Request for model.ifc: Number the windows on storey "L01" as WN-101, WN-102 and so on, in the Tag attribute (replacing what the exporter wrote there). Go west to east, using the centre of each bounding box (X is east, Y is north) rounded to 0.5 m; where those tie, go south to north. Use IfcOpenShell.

First a look at what the model holds.

```python
import ifcopenshell
import ifcopenshell.util.element
import ifcopenshell.util.placement

model = ifcopenshell.open("model.ifc")
print(model.schema)
storey = next(s for s in model.by_type("IfcBuildingStorey") if s.Name == "L01")
windows = [e for e in ifcopenshell.util.element.get_decomposition(storey) if e.is_a("IfcWindow")]
for e in sorted(windows, key=lambda e: e.id()):
    origin = ifcopenshell.util.placement.get_local_placement(e.ObjectPlacement)[:3, 3]
    print(e.id(), e.Tag, e.Name, origin.round(2) + 0.0, sep=" | ")
```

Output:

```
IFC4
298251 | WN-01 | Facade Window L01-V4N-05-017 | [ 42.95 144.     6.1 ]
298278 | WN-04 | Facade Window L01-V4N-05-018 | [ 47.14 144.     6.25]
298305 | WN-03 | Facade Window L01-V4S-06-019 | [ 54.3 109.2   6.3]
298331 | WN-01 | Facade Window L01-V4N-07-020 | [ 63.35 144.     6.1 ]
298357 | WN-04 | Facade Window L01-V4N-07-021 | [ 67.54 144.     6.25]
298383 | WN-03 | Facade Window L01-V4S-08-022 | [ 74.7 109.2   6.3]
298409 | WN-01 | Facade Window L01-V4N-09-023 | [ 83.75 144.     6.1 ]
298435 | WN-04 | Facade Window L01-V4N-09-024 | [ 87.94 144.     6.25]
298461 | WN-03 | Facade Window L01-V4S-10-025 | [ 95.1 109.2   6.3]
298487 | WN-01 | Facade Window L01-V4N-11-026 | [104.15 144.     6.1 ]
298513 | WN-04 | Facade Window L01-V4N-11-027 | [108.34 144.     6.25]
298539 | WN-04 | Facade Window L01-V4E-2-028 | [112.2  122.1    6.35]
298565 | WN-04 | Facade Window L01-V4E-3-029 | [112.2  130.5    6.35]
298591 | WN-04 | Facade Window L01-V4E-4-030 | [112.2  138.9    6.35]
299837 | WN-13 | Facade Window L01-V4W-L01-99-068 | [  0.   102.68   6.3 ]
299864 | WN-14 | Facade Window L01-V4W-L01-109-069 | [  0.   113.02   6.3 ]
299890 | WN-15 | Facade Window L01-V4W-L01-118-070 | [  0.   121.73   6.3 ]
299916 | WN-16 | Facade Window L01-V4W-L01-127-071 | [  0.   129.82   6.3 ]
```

```python
import ifcopenshell
import ifcopenshell.geom
import ifcopenshell.util.element
import ifcopenshell.util.shape

model = ifcopenshell.open("model.ifc")
settings = ifcopenshell.geom.settings()
settings.set("use-world-coords", True)


def centre(element):
    shape = ifcopenshell.geom.create_shape(settings, element)
    return ifcopenshell.util.shape.get_bbox_centroid(shape.geometry)


storey = next(s for s in model.by_type("IfcBuildingStorey") if s.Name == "L01")
windows = [e for e in ifcopenshell.util.element.get_decomposition(storey) if e.is_a("IfcWindow")]

# Insertion points can sit at a corner or the storey origin, so sort by the geometry (in metres).
centres = {e: centre(e) for e in windows}
windows.sort(key=lambda e: (round(centres[e][0] / 0.5), centres[e][1]))

for i, e in enumerate(windows, start=1):
    number = f"WN-1{i:02d}"
    e.Tag = number
    print(e.id(), number)

model.write("model_edited.ifc")
```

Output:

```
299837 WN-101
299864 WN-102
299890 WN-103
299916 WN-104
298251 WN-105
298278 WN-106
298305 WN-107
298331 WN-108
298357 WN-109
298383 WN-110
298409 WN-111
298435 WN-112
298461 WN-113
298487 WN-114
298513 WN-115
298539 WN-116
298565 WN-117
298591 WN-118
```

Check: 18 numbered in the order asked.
